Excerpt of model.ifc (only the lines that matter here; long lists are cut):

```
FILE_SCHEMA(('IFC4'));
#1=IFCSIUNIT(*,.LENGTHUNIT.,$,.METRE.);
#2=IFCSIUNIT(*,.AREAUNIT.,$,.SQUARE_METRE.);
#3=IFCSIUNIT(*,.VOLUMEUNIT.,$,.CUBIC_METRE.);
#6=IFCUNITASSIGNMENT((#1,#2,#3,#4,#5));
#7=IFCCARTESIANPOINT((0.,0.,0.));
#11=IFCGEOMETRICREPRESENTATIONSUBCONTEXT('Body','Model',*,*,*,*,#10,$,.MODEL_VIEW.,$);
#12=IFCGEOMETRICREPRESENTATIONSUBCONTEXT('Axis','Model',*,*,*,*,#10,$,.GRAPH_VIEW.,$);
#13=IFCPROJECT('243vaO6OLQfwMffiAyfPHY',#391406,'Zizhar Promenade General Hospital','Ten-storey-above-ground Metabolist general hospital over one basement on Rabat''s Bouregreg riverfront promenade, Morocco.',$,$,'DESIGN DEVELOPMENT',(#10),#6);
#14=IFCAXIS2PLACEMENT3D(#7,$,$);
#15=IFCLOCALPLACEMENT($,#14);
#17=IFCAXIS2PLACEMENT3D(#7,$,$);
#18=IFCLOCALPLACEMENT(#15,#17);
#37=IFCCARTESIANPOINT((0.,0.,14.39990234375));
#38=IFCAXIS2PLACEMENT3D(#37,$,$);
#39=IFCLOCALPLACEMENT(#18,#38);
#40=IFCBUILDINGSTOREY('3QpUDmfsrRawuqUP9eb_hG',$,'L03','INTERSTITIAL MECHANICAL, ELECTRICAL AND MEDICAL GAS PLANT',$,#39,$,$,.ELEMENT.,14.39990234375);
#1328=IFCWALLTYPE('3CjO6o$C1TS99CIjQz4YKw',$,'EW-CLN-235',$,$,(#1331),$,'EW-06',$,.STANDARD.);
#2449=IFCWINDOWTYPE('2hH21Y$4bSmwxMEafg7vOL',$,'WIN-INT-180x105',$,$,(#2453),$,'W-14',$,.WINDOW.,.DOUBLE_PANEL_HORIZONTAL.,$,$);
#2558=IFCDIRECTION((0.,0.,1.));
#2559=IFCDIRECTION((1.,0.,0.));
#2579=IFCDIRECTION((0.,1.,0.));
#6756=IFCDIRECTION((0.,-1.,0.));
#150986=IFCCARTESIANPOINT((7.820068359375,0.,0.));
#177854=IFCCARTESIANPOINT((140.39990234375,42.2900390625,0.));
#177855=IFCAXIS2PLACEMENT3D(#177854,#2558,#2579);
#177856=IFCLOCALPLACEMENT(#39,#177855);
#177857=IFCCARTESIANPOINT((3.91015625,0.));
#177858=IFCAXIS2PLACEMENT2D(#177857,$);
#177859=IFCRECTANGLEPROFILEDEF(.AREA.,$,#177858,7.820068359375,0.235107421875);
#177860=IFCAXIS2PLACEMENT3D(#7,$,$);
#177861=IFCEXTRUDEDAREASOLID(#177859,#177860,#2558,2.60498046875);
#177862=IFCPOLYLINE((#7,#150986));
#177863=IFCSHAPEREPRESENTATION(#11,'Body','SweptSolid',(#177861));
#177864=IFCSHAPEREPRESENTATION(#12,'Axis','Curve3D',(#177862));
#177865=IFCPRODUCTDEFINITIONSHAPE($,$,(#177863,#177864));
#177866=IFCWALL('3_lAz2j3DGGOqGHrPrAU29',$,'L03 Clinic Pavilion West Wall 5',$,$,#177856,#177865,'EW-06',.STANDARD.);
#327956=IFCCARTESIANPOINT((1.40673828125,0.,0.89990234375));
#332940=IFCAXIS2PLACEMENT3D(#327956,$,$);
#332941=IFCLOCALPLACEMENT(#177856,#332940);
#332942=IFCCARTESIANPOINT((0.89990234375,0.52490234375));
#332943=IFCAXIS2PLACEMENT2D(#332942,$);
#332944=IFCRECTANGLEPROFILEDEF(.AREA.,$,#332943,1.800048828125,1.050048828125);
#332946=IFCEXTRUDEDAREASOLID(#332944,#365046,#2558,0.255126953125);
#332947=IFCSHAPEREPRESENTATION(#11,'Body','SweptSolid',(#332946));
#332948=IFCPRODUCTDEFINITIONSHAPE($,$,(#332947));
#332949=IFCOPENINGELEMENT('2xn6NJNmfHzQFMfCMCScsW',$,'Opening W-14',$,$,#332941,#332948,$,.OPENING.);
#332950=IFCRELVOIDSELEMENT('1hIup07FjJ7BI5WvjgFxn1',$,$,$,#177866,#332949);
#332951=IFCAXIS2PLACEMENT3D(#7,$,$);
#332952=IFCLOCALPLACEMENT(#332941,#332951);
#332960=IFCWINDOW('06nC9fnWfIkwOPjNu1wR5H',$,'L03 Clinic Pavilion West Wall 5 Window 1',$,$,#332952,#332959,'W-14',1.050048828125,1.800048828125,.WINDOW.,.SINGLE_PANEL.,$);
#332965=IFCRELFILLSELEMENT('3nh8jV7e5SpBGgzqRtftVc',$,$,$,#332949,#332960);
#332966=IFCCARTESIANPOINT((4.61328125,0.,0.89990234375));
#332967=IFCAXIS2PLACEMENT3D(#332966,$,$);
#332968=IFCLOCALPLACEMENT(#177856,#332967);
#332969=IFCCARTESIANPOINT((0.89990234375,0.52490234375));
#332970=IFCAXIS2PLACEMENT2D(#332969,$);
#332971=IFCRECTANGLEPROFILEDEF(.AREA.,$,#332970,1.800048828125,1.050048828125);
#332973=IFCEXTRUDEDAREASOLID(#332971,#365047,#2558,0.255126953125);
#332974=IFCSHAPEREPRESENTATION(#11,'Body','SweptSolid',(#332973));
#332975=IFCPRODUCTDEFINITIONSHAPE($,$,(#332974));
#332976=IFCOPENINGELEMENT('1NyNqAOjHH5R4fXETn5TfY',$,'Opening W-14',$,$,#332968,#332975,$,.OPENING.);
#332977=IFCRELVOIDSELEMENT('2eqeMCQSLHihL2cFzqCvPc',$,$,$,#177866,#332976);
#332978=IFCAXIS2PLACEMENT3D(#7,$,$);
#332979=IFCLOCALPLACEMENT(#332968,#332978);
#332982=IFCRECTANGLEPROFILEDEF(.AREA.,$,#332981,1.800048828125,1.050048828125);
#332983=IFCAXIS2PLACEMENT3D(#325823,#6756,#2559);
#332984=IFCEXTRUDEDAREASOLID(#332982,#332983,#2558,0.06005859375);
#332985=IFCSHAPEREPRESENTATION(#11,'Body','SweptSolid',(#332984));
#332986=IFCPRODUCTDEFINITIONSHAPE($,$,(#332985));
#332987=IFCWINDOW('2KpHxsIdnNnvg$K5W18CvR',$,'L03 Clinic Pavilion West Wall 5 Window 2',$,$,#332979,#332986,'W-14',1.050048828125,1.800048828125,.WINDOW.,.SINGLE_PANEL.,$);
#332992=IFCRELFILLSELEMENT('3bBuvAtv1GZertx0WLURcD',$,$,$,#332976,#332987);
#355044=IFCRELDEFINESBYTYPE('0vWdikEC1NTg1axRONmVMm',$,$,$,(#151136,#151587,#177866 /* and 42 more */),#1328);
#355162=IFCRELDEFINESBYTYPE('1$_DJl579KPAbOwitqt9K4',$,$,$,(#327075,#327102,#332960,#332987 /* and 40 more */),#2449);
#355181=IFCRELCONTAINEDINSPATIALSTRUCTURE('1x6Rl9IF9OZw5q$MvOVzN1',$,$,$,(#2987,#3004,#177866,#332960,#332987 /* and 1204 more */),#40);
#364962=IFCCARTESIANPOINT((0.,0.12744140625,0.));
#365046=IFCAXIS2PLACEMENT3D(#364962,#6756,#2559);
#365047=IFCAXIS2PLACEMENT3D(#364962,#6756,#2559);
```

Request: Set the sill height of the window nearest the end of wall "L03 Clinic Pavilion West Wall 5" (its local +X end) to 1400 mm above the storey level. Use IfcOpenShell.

```python
import numpy as np
import ifcopenshell
import ifcopenshell.api.geometry
import ifcopenshell.geom
import ifcopenshell.util.element
import ifcopenshell.util.placement
import ifcopenshell.util.shape
import ifcopenshell.util.unit

model = ifcopenshell.open("model.ifc")
unit_scale = ifcopenshell.util.unit.calculate_unit_scale(model)

window = model.by_guid("2KpHxsIdnNnvg$K5W18CvR")
opening = window.FillsVoids[0].RelatingOpeningElement
storey = ifcopenshell.util.element.get_container(window, ifc_class="IfcBuildingStorey")
level = ifcopenshell.util.placement.get_local_placement(storey.ObjectPlacement)[2, 3]

# The opening's origin need not be at the sill, so measure its lowest point.
shape = ifcopenshell.geom.create_shape(ifcopenshell.geom.settings(), opening)
bottom = ifcopenshell.util.shape.get_shape_bottom_elevation(shape, shape.geometry) / unit_scale
dz = level + 1.4 - bottom

shift = np.array([0.0, 0.0, dz])
# The window is placed relative to its opening, so it follows when the opening moves.
matrix = ifcopenshell.util.placement.get_local_placement(opening.ObjectPlacement)
matrix[:3, 3] += shift
ifcopenshell.api.geometry.edit_object_placement(
    model, product=opening, matrix=matrix, is_si=False, should_transform_children=True
)

print(f"moved by {dz * unit_scale:+.3f} m")

model.write("model_v2.ifc")
```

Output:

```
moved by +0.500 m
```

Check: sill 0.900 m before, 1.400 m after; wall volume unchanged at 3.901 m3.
